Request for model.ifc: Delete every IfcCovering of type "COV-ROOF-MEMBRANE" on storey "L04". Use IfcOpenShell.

First a look at what the model holds.

```python
import ifcopenshell
import ifcopenshell.util.element

model = ifcopenshell.open("model.ifc")
print(model.schema)
storey = next(s for s in model.by_type("IfcBuildingStorey") if s.Name == "L04")
coverings = [e for e in ifcopenshell.util.element.get_decomposition(storey) if e.is_a("IfcCovering")]
seen = {}
for e in coverings:
    element_type = ifcopenshell.util.element.get_type(e)
    name = element_type.Name if element_type not in (None, e) else None
    seen[name] = seen.get(name, 0) + 1
for name, count in sorted(seen.items(), key=str):
    print(count, "x", name)
```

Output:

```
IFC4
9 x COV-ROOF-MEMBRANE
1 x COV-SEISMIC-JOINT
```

```python
import ifcopenshell
import ifcopenshell.api.root
import ifcopenshell.util.element

model = ifcopenshell.open("model.ifc")

storey = next(s for s in model.by_type("IfcBuildingStorey") if s.Name == "L04")
coverings = [e for e in ifcopenshell.util.element.get_decomposition(storey) if e.is_a("IfcCovering")]
targets = [e for e in coverings if (t := ifcopenshell.util.element.get_type(e)) not in (None, e) and t.Name == "COV-ROOF-MEMBRANE"]

for e in targets:
    ifcopenshell.api.root.remove_product(model, product=e)
print(len(targets), "removed")

model.write("model-out.ifc")
```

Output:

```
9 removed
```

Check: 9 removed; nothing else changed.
